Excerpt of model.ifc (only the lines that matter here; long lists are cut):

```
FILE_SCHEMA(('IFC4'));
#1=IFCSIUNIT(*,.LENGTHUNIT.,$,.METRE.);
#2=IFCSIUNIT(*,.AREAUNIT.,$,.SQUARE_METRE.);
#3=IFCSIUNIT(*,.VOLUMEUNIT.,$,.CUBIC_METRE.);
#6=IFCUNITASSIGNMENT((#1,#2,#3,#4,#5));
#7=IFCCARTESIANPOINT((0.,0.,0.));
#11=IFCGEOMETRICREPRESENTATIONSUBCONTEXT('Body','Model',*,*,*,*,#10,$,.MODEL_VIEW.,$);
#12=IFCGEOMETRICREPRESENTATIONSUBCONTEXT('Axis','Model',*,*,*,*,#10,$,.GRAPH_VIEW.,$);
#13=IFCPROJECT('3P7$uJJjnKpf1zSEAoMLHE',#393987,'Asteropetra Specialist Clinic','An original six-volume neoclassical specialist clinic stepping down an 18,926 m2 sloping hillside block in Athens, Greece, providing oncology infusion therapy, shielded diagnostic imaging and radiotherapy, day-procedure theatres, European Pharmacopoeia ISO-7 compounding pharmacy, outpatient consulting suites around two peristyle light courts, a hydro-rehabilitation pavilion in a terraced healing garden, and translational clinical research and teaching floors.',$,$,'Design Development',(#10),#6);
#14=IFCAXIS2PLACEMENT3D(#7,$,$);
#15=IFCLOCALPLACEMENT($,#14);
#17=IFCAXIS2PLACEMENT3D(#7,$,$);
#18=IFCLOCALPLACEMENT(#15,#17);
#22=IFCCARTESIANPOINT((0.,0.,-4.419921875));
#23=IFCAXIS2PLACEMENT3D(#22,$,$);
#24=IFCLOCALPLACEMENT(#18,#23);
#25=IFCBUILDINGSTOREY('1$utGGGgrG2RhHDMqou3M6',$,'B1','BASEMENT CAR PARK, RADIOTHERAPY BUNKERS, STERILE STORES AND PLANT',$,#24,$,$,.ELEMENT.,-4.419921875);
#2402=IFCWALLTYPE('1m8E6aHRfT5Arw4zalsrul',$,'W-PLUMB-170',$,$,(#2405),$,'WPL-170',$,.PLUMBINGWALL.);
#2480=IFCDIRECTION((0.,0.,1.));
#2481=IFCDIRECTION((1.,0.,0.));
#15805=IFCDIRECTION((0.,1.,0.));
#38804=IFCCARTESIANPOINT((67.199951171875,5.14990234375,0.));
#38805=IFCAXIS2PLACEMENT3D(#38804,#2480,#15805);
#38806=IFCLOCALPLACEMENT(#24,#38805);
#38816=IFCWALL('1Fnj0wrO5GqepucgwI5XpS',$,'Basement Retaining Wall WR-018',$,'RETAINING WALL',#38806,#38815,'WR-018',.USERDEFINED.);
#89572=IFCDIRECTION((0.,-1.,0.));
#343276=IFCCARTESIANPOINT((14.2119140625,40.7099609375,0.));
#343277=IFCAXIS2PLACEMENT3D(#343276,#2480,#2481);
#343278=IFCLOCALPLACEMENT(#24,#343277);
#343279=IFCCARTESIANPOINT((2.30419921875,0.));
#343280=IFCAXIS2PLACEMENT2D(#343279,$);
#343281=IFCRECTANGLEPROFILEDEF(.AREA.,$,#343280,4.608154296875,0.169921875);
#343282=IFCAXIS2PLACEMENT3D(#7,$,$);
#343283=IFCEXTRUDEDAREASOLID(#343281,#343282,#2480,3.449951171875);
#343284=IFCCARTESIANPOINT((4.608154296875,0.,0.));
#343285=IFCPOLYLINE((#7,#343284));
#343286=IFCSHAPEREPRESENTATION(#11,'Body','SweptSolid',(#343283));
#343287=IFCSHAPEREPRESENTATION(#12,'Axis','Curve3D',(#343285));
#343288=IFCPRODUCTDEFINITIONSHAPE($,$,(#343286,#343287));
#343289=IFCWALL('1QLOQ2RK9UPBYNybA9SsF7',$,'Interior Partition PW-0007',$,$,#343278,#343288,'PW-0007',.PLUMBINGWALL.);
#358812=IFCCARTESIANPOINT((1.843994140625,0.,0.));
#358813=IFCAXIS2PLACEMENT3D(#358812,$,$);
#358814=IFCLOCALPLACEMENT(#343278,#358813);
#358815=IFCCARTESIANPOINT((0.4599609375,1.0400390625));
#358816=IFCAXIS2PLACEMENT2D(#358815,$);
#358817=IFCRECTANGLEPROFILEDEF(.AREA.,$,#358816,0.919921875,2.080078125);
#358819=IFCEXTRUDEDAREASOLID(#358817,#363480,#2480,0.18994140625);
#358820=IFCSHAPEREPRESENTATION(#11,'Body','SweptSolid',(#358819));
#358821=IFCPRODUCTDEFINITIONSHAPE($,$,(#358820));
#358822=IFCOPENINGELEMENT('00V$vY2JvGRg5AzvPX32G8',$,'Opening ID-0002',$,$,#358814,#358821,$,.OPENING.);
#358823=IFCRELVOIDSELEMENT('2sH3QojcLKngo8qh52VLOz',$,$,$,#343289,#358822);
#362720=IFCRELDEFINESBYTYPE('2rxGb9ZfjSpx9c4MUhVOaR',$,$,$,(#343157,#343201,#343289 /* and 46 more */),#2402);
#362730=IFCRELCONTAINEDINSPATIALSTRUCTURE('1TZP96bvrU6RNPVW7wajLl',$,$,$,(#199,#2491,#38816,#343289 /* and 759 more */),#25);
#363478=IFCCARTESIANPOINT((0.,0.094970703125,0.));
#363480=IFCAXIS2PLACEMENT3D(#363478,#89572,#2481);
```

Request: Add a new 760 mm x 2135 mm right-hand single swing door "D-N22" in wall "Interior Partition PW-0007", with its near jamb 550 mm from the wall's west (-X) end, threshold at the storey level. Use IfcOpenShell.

```python
import numpy as np
import ifcopenshell
import ifcopenshell.api.feature
import ifcopenshell.api.geometry
import ifcopenshell.api.root
import ifcopenshell.api.spatial
import ifcopenshell.geom
import ifcopenshell.util.element
import ifcopenshell.util.placement
import ifcopenshell.util.representation
import ifcopenshell.util.shape
import ifcopenshell.util.unit

model = ifcopenshell.open("model.ifc")
unit_scale = ifcopenshell.util.unit.calculate_unit_scale(model)
settings = ifcopenshell.geom.settings()


def volume(element):
    """Net volume in cubic metres, openings subtracted."""
    shape = ifcopenshell.geom.create_shape(settings, element)
    return ifcopenshell.util.shape.get_volume(shape.geometry)


wall = model.by_guid("1QLOQ2RK9UPBYNybA9SsF7")
storey = ifcopenshell.util.element.get_container(wall, ifc_class="IfcBuildingStorey")
context = ifcopenshell.util.representation.get_context(model, "Model", "Body", "MODEL_VIEW")
before = volume(wall)

width, height, from_end, sill = 0.76, 2.135, 0.55, 0.0  # metres

# The wall runs along its own X axis, and the end named is its -X end.
wall_shape = ifcopenshell.geom.create_shape(settings, wall)
x, y, z = ifcopenshell.util.shape.get_vertices(wall_shape.geometry).T
start = x.min() + from_end
face, thickness = float(y.min()), float(y.max() - y.min())
wall_matrix = ifcopenshell.util.placement.get_local_placement(wall.ObjectPlacement)
level = ifcopenshell.util.placement.get_local_placement(storey.ObjectPlacement)[2, 3]


def in_wall(x, y):
    """Placement at x, y metres in the wall's axes, at sill height."""
    matrix = wall_matrix.copy()
    matrix[:, 3] = wall_matrix @ np.array([x / unit_scale, y / unit_scale, 0.0, 1.0])
    matrix[2, 3] = level + sill / unit_scale
    return matrix


# Opening: a box that overshoots both wall faces by 50 mm.
opening = ifcopenshell.api.root.create_entity(model, ifc_class="IfcOpeningElement", predefined_type="OPENING")
box = ifcopenshell.api.geometry.add_wall_representation(
    model, context=context, length=width, height=height, thickness=thickness + 0.1
)
ifcopenshell.api.geometry.assign_representation(model, product=opening, representation=box)
ifcopenshell.api.geometry.edit_object_placement(model, product=opening, matrix=in_wall(start, face - 0.05), is_si=False)
ifcopenshell.api.feature.add_feature(model, feature=opening, element=wall)

door = ifcopenshell.api.root.create_entity(model, ifc_class="IfcDoor", name="D-N22", predefined_type="DOOR")
door.OverallWidth, door.OverallHeight = width / unit_scale, height / unit_scale
door.OperationType = "SINGLE_SWING_RIGHT"
body = ifcopenshell.api.geometry.add_door_representation(
    model,
    context=context,
    overall_width=door.OverallWidth,
    overall_height=door.OverallHeight,
    operation_type="SINGLE_SWING_RIGHT",
    lining_properties={"LiningDepth": thickness / unit_scale, "ThresholdDepth": thickness / unit_scale},
)
ifcopenshell.api.geometry.assign_representation(model, product=door, representation=body)
ifcopenshell.api.spatial.assign_container(model, products=[door], relating_structure=storey)
ifcopenshell.api.feature.add_filling(model, opening=opening, element=door)

# The lining spans the wall, so the door starts at the wall face.
ifcopenshell.api.geometry.edit_object_placement(model, product=door, matrix=in_wall(start, face), is_si=False)

after = volume(wall)

print(f"wall volume {before:.3f} -> {after:.3f} m3")

model.write("model_rev.ifc")
```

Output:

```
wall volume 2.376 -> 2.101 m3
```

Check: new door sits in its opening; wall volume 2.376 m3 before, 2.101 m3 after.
